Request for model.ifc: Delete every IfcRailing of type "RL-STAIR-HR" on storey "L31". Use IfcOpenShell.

First a look at what the model holds.

```python
import ifcopenshell
import ifcopenshell.util.element

model = ifcopenshell.open("model.ifc")
print(model.schema)
storey = next(s for s in model.by_type("IfcBuildingStorey") if s.Name == "L31")
railings = [e for e in ifcopenshell.util.element.get_decomposition(storey) if e.is_a("IfcRailing")]
seen = {}
for e in railings:
    element_type = ifcopenshell.util.element.get_type(e)
    name = element_type.Name if element_type not in (None, e) else None
    seen[name] = seen.get(name, 0) + 1
for name, count in sorted(seen.items(), key=str):
    print(count, "x", name)
```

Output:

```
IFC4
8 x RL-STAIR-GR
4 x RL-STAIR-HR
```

```python
import ifcopenshell
import ifcopenshell.api.root
import ifcopenshell.util.element

model = ifcopenshell.open("model.ifc")

storey = next(s for s in model.by_type("IfcBuildingStorey") if s.Name == "L31")
railings = [e for e in ifcopenshell.util.element.get_decomposition(storey) if e.is_a("IfcRailing")]
targets = [e for e in railings if (t := ifcopenshell.util.element.get_type(e)) not in (None, e) and t.Name == "RL-STAIR-HR"]

for e in targets:
    ifcopenshell.api.root.remove_product(model, product=e)
print(len(targets), "removed")

model.write("model_updated.ifc")
```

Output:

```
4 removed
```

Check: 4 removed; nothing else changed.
